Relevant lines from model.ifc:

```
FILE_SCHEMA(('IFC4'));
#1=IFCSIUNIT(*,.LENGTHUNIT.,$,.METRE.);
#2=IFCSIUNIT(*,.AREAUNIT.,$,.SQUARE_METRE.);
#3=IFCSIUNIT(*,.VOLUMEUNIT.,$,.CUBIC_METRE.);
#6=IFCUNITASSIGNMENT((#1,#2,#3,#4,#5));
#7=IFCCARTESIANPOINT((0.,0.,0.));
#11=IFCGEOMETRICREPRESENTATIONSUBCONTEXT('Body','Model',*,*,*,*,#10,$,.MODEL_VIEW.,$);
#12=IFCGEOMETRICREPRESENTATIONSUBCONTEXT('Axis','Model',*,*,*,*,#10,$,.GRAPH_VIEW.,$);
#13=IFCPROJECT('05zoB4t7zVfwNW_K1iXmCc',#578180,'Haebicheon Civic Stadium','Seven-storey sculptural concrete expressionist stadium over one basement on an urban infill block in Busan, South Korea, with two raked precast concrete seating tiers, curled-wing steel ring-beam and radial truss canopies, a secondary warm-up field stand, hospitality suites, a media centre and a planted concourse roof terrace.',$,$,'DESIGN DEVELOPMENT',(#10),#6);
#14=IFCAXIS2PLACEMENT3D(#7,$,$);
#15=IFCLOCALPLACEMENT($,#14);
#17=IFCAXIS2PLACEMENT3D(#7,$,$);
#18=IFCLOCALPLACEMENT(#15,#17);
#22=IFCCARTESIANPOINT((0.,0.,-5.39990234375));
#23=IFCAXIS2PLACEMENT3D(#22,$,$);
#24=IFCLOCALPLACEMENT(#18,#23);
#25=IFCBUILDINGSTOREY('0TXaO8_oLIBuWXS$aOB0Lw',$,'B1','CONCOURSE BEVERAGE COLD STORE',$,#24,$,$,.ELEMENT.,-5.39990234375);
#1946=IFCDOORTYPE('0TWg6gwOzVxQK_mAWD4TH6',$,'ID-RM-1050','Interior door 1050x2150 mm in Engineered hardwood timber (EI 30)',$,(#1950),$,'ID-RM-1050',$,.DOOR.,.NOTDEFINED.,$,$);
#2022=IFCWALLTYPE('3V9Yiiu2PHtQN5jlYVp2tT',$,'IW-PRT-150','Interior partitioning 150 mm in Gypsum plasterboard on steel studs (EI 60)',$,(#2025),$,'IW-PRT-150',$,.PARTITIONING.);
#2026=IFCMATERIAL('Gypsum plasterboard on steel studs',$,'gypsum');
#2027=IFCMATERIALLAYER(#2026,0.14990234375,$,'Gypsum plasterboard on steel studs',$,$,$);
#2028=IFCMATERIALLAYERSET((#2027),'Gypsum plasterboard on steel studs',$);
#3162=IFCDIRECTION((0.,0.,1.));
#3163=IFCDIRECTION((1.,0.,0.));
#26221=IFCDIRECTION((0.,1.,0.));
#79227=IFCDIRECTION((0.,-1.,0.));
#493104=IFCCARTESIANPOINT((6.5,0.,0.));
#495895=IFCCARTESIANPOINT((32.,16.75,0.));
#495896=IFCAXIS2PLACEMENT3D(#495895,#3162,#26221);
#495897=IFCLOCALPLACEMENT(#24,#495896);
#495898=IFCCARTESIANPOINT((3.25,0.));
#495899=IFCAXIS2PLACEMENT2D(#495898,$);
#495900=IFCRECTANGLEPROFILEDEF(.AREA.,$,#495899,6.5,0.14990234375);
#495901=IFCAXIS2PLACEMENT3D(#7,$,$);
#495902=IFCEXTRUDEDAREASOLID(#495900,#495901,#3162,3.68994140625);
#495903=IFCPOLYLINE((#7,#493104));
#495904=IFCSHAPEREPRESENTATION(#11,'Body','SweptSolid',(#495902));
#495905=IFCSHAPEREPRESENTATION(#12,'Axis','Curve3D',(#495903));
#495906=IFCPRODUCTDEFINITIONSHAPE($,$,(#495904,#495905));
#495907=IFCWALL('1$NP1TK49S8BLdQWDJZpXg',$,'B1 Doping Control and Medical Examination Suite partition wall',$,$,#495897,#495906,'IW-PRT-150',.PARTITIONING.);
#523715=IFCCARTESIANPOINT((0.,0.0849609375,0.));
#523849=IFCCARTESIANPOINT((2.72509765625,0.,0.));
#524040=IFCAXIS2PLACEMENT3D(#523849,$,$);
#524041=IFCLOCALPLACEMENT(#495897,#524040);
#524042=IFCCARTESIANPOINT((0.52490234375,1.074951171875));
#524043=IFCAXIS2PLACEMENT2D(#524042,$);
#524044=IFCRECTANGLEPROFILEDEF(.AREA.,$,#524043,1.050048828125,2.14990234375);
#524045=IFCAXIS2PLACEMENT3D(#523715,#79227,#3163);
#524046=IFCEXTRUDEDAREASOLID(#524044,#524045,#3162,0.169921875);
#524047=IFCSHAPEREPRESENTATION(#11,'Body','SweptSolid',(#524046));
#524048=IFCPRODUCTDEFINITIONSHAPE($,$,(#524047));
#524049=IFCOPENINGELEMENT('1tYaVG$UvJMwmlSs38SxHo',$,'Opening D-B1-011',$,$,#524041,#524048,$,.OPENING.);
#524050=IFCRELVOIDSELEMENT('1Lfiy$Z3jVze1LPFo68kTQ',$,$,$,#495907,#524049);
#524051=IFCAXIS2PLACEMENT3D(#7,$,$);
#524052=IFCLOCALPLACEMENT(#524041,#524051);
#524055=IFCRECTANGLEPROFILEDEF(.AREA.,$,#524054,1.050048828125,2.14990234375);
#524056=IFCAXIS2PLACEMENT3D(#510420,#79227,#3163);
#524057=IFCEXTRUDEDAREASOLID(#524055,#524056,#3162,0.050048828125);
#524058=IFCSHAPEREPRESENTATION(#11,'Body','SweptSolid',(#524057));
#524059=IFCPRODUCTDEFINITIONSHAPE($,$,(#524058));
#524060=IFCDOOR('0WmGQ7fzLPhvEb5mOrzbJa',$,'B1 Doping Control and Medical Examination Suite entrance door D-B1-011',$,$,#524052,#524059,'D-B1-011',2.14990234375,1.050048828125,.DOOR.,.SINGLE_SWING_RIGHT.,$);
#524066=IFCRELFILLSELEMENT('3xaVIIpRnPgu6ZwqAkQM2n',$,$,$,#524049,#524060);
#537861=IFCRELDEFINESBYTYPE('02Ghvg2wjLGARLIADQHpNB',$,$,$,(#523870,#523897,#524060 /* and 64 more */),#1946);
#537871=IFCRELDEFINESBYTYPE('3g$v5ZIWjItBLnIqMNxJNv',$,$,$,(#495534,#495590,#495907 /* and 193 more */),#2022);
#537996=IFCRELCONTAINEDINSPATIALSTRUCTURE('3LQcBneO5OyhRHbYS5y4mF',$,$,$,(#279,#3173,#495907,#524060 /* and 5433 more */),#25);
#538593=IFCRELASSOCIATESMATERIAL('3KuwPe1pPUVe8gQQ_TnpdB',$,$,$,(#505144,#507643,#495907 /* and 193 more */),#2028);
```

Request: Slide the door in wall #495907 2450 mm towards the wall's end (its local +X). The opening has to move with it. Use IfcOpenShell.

```python
import ifcopenshell
import ifcopenshell.api.geometry
import ifcopenshell.util.placement
import ifcopenshell.util.unit

model = ifcopenshell.open("model.ifc")
unit_scale = ifcopenshell.util.unit.calculate_unit_scale(model)

door = model.by_guid("0WmGQ7fzLPhvEb5mOrzbJa")
opening = door.FillsVoids[0].RelatingOpeningElement
wall = opening.VoidsElements[0].RelatingBuildingElement

wall_matrix = ifcopenshell.util.placement.get_local_placement(wall.ObjectPlacement)
shift = wall_matrix[:3, 0] * 2.45 / unit_scale
before = ifcopenshell.util.placement.get_local_placement(door.ObjectPlacement)[:3, 3].copy()

# The door is placed relative to its opening, so it follows when the opening moves.
matrix = ifcopenshell.util.placement.get_local_placement(opening.ObjectPlacement)
matrix[:3, 3] += shift
ifcopenshell.api.geometry.edit_object_placement(
    model, product=opening, matrix=matrix, is_si=False, should_transform_children=True
)

after = ifcopenshell.util.placement.get_local_placement(door.ObjectPlacement)[:3, 3]
print("door moved by", (after - before).round(3) + 0.0)

model.write("model_v2.ifc")
```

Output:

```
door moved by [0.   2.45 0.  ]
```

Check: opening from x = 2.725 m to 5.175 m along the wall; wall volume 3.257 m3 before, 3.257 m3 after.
